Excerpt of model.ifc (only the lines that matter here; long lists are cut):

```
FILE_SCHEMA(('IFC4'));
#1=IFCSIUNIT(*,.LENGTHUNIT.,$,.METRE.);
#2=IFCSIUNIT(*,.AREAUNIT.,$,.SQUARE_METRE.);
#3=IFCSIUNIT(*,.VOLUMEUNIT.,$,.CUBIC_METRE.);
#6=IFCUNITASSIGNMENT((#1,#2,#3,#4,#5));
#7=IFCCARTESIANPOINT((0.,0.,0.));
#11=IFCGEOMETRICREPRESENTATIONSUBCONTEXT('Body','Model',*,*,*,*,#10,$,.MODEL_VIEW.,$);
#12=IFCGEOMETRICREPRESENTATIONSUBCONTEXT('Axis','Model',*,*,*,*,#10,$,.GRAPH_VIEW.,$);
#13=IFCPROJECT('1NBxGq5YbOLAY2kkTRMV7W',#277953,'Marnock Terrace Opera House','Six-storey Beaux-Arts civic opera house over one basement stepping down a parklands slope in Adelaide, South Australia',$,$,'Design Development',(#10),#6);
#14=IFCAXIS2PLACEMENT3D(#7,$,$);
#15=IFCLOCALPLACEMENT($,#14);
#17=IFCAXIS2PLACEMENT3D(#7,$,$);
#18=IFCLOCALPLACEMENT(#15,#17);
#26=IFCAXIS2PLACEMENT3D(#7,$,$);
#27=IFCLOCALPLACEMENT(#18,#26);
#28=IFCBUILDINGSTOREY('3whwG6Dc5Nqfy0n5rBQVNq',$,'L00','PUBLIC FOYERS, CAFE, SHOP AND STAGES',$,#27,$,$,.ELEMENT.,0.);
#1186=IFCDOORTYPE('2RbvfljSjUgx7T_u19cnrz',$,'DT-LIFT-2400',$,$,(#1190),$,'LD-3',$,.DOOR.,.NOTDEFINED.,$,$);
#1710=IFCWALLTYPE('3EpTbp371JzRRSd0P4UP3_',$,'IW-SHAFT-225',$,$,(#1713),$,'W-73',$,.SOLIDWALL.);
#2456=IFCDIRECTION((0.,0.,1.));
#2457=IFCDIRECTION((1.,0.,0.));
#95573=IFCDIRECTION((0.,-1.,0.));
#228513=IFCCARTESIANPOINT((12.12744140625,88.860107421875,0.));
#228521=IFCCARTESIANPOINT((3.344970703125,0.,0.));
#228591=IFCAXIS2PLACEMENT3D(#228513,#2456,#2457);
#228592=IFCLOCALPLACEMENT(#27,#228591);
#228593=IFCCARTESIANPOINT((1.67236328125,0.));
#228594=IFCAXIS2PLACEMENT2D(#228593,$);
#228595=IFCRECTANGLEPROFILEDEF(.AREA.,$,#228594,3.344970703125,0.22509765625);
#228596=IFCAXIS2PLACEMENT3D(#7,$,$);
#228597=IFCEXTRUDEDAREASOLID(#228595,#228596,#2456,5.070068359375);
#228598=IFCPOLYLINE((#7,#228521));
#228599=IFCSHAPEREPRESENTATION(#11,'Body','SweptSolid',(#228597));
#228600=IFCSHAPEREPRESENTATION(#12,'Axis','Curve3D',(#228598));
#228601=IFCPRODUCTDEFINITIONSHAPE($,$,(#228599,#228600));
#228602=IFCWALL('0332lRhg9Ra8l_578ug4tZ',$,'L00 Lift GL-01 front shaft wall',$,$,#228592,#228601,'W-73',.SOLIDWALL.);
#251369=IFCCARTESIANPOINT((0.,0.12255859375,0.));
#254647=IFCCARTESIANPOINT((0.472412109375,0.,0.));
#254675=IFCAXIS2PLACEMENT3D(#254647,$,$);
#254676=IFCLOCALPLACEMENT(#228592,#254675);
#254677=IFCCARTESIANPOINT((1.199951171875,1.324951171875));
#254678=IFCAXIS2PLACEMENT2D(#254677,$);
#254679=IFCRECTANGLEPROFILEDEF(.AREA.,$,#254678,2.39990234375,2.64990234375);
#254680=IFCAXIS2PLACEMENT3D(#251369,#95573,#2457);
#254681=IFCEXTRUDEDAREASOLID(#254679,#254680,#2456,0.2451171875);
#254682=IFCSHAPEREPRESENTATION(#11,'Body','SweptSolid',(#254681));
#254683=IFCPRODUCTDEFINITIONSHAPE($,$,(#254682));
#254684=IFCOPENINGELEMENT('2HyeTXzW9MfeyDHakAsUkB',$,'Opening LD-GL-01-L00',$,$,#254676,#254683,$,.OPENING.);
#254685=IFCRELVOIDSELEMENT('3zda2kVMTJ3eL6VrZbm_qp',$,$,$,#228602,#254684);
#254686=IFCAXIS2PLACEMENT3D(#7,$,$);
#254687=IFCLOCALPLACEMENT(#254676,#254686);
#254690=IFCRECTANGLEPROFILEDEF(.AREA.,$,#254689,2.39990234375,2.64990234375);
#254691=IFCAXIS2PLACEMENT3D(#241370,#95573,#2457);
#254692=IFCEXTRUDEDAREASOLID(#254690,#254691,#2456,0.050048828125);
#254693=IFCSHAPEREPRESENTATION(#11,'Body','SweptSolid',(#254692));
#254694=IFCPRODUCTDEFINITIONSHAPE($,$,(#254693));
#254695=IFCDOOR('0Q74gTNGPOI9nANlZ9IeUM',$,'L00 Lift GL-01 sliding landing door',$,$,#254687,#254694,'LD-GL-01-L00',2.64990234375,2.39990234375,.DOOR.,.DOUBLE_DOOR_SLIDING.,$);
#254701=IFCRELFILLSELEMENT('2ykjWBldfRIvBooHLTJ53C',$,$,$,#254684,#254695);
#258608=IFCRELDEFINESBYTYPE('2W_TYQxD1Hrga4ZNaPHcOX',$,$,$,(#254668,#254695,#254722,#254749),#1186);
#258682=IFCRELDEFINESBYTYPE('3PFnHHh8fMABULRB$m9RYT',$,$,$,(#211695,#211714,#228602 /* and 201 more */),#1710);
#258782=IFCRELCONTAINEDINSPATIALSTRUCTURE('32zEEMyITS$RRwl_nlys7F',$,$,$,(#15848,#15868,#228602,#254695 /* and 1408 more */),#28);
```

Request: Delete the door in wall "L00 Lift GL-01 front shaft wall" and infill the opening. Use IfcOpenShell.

```python
import ifcopenshell
import ifcopenshell.api.feature
import ifcopenshell.api.root
import ifcopenshell.geom
import ifcopenshell.util.shape

model = ifcopenshell.open("model.ifc")
settings = ifcopenshell.geom.settings()


def volume(element):
    """Net volume in cubic metres, openings subtracted."""
    shape = ifcopenshell.geom.create_shape(settings, element)
    return ifcopenshell.util.shape.get_volume(shape.geometry)


door = model.by_guid("0Q74gTNGPOI9nANlZ9IeUM")
opening = door.FillsVoids[0].RelatingOpeningElement
wall = opening.VoidsElements[0].RelatingBuildingElement
before = volume(wall)

ifcopenshell.api.root.remove_product(model, product=door)
ifcopenshell.api.feature.remove_feature(model, feature=opening)

after = volume(wall)

print(f"wall volume {before:.3f} -> {after:.3f} m3")

model.write("model_edited.ifc")
```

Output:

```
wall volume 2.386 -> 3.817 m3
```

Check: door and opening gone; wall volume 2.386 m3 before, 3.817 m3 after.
